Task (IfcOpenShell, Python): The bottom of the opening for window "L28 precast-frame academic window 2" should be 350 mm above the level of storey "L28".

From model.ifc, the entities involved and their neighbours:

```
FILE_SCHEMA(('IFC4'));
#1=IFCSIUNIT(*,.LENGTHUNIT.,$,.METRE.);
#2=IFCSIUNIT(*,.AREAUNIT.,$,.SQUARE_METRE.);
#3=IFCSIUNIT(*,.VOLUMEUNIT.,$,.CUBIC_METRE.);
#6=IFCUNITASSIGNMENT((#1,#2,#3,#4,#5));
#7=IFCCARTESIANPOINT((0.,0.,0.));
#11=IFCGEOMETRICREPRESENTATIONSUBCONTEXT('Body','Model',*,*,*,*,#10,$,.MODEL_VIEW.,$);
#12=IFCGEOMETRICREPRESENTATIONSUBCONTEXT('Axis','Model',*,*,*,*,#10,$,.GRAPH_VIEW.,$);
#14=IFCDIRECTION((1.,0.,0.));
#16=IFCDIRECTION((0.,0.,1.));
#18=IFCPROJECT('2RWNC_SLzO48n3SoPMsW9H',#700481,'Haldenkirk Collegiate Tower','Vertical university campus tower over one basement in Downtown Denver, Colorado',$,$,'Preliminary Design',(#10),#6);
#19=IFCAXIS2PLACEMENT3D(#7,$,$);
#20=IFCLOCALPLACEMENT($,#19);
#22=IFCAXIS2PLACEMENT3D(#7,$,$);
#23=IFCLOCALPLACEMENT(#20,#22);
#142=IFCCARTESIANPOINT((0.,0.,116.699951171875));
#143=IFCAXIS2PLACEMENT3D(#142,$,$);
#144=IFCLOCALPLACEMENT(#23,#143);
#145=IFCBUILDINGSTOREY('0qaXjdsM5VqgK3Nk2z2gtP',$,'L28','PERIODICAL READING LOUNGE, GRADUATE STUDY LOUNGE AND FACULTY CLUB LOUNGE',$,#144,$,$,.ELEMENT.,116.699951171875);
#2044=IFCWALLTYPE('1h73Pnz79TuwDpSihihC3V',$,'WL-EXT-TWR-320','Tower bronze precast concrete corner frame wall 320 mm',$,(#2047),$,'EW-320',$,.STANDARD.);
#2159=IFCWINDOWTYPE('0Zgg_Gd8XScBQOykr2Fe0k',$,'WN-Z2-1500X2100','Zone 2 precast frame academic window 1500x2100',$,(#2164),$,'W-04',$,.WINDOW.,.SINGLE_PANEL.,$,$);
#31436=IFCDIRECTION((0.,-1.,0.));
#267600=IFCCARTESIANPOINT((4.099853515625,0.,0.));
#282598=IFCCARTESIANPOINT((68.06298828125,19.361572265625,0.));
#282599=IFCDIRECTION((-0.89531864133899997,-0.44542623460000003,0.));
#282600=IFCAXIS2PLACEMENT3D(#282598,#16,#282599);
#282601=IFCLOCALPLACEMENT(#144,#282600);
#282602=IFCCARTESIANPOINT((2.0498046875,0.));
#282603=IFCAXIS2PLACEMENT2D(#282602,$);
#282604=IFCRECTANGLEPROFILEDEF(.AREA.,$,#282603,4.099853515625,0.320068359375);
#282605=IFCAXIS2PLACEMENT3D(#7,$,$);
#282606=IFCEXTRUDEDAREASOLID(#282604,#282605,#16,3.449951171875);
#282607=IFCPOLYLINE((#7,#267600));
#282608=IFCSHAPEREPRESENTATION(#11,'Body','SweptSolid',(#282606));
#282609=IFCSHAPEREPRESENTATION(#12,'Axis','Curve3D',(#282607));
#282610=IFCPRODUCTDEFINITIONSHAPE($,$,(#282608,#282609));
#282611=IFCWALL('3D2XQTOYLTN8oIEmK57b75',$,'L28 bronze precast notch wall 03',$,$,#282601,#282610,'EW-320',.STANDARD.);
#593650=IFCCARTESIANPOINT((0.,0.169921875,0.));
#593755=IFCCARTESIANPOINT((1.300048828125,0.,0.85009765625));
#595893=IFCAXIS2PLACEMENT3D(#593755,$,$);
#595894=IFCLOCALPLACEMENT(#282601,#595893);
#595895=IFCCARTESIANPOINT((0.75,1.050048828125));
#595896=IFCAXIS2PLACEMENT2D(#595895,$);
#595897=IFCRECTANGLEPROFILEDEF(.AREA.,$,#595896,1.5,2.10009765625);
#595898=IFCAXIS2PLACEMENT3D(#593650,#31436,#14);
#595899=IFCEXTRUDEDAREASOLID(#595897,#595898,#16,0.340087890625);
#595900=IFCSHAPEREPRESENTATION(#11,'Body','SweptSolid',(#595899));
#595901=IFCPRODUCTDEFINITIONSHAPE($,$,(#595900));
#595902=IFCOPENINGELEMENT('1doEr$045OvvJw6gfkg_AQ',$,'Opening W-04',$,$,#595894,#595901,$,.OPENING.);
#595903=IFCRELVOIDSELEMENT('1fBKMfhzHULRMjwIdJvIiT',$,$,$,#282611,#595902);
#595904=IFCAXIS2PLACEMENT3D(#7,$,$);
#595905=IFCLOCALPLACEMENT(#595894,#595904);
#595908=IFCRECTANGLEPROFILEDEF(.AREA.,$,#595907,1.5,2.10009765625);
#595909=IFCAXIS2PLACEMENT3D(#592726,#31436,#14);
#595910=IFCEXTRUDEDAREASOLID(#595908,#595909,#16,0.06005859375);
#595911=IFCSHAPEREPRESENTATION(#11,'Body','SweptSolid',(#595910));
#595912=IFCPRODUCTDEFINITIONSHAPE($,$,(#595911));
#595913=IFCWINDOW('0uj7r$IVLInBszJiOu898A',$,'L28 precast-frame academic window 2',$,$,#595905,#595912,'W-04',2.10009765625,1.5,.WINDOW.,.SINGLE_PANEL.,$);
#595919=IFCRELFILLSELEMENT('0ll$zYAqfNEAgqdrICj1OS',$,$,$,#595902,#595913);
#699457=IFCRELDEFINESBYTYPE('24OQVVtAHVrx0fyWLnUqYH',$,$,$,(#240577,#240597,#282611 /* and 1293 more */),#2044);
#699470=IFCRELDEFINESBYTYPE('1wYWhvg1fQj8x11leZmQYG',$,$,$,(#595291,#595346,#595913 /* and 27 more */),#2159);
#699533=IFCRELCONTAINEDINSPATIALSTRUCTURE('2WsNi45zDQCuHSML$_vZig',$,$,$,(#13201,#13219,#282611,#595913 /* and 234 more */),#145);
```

```python
import numpy as np
import ifcopenshell
import ifcopenshell.api.geometry
import ifcopenshell.geom
import ifcopenshell.util.element
import ifcopenshell.util.placement
import ifcopenshell.util.shape
import ifcopenshell.util.unit

model = ifcopenshell.open("model.ifc")
unit_scale = ifcopenshell.util.unit.calculate_unit_scale(model)

window = model.by_guid("0uj7r$IVLInBszJiOu898A")
opening = window.FillsVoids[0].RelatingOpeningElement
storey = ifcopenshell.util.element.get_container(window, ifc_class="IfcBuildingStorey")
level = ifcopenshell.util.placement.get_local_placement(storey.ObjectPlacement)[2, 3]

# The opening's origin need not be at the sill, so measure its lowest point.
shape = ifcopenshell.geom.create_shape(ifcopenshell.geom.settings(), opening)
bottom = ifcopenshell.util.shape.get_shape_bottom_elevation(shape, shape.geometry) / unit_scale
dz = level + 0.35 - bottom

shift = np.array([0.0, 0.0, dz])
# The window is placed relative to its opening, so it follows when the opening moves.
matrix = ifcopenshell.util.placement.get_local_placement(opening.ObjectPlacement)
matrix[:3, 3] += shift
ifcopenshell.api.geometry.edit_object_placement(
    model, product=opening, matrix=matrix, is_si=False, should_transform_children=True
)

print(f"moved by {dz * unit_scale:+.3f} m")

model.write("model_updated.ifc")
```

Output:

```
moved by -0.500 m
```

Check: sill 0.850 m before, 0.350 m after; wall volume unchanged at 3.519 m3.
